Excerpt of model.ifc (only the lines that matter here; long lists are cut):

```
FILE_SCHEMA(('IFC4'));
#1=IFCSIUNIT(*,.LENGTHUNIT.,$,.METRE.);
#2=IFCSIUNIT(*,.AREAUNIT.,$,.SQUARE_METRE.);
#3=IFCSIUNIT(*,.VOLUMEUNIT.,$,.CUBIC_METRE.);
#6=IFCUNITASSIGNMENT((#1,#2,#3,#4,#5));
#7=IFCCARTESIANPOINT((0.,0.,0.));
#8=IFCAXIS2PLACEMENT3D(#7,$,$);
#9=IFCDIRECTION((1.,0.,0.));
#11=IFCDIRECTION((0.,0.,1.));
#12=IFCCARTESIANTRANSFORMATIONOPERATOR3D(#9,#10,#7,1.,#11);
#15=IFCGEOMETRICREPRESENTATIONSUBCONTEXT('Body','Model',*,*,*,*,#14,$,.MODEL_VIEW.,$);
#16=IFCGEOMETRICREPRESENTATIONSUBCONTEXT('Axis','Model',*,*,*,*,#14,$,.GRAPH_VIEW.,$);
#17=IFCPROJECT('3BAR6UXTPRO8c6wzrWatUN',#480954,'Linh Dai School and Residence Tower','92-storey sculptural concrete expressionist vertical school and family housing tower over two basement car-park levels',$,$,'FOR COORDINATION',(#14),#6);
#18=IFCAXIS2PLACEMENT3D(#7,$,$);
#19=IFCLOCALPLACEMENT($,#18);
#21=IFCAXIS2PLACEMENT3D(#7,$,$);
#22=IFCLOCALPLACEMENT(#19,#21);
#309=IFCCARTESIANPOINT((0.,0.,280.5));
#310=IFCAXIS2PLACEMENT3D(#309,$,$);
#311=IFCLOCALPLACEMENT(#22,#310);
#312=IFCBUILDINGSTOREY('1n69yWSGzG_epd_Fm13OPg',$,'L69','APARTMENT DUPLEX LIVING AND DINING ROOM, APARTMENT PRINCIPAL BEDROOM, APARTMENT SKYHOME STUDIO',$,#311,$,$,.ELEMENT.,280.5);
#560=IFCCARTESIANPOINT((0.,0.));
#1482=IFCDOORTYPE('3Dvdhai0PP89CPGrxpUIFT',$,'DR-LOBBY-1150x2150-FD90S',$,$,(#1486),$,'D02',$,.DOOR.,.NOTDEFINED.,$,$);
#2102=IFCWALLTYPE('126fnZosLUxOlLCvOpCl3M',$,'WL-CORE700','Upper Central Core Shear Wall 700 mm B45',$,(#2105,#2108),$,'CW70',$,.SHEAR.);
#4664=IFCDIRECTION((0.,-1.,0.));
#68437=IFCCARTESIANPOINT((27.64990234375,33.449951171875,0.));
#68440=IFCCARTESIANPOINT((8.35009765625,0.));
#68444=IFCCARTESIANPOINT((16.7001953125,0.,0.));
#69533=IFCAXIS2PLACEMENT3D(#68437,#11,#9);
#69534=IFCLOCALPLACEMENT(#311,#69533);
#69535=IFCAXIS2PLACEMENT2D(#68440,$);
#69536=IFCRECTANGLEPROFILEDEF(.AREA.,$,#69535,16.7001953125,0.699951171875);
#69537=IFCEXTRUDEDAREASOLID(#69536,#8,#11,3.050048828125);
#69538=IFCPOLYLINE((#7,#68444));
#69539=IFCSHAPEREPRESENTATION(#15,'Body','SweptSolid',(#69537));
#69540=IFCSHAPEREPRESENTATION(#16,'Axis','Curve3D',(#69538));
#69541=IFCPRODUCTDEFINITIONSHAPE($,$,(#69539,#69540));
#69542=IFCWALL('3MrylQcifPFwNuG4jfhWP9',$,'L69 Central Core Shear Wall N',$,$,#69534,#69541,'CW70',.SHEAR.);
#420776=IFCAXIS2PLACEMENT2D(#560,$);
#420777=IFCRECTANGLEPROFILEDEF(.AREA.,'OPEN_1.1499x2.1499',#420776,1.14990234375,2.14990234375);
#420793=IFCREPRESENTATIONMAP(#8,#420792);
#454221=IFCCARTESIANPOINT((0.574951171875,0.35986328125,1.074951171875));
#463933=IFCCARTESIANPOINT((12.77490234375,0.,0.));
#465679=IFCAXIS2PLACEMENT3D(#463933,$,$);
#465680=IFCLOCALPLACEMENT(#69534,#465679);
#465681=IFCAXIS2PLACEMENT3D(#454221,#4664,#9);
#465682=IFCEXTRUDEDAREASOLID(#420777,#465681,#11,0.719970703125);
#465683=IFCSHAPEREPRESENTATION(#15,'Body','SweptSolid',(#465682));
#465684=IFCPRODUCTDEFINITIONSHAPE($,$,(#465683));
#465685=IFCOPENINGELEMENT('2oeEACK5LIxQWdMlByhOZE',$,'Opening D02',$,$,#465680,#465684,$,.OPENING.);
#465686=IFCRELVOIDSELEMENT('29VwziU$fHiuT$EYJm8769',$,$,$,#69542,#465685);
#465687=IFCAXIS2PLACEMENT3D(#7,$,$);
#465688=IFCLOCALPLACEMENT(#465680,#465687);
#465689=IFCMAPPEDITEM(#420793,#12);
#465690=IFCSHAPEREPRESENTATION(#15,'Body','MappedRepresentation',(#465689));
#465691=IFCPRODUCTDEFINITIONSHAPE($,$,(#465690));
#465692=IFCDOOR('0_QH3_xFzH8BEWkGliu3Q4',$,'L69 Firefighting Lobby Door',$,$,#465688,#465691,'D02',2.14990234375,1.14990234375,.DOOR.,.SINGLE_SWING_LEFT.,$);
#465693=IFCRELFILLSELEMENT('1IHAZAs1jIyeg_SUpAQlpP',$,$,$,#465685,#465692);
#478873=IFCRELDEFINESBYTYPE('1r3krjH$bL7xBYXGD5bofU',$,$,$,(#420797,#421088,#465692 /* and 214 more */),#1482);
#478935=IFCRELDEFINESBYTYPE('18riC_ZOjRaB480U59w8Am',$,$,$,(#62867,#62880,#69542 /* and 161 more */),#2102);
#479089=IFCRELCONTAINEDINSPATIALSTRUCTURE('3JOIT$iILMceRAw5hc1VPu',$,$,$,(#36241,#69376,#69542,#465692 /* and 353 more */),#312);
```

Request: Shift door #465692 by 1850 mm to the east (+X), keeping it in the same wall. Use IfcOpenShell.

```python
import ifcopenshell
import ifcopenshell.api.geometry
import ifcopenshell.util.placement

model = ifcopenshell.open("model.ifc")

door = model.by_guid("0_QH3_xFzH8BEWkGliu3Q4")
opening = door.FillsVoids[0].RelatingOpeningElement
wall = opening.VoidsElements[0].RelatingBuildingElement

wall_matrix = ifcopenshell.util.placement.get_local_placement(wall.ObjectPlacement)
shift = wall_matrix[:3, 0] * 1.85
before = ifcopenshell.util.placement.get_local_placement(door.ObjectPlacement)[:3, 3].copy()

# The door is placed relative to its opening, so it follows when the opening moves.
matrix = ifcopenshell.util.placement.get_local_placement(opening.ObjectPlacement)
matrix[:3, 3] += shift
ifcopenshell.api.geometry.edit_object_placement(
    model, product=opening, matrix=matrix, is_si=False, should_transform_children=True
)

after = ifcopenshell.util.placement.get_local_placement(door.ObjectPlacement)[:3, 3]
print("door moved by", (after - before).round(3) + 0.0)

model.write("model-out.ifc")
```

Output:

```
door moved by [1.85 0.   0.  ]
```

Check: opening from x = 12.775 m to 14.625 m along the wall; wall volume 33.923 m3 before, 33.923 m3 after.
